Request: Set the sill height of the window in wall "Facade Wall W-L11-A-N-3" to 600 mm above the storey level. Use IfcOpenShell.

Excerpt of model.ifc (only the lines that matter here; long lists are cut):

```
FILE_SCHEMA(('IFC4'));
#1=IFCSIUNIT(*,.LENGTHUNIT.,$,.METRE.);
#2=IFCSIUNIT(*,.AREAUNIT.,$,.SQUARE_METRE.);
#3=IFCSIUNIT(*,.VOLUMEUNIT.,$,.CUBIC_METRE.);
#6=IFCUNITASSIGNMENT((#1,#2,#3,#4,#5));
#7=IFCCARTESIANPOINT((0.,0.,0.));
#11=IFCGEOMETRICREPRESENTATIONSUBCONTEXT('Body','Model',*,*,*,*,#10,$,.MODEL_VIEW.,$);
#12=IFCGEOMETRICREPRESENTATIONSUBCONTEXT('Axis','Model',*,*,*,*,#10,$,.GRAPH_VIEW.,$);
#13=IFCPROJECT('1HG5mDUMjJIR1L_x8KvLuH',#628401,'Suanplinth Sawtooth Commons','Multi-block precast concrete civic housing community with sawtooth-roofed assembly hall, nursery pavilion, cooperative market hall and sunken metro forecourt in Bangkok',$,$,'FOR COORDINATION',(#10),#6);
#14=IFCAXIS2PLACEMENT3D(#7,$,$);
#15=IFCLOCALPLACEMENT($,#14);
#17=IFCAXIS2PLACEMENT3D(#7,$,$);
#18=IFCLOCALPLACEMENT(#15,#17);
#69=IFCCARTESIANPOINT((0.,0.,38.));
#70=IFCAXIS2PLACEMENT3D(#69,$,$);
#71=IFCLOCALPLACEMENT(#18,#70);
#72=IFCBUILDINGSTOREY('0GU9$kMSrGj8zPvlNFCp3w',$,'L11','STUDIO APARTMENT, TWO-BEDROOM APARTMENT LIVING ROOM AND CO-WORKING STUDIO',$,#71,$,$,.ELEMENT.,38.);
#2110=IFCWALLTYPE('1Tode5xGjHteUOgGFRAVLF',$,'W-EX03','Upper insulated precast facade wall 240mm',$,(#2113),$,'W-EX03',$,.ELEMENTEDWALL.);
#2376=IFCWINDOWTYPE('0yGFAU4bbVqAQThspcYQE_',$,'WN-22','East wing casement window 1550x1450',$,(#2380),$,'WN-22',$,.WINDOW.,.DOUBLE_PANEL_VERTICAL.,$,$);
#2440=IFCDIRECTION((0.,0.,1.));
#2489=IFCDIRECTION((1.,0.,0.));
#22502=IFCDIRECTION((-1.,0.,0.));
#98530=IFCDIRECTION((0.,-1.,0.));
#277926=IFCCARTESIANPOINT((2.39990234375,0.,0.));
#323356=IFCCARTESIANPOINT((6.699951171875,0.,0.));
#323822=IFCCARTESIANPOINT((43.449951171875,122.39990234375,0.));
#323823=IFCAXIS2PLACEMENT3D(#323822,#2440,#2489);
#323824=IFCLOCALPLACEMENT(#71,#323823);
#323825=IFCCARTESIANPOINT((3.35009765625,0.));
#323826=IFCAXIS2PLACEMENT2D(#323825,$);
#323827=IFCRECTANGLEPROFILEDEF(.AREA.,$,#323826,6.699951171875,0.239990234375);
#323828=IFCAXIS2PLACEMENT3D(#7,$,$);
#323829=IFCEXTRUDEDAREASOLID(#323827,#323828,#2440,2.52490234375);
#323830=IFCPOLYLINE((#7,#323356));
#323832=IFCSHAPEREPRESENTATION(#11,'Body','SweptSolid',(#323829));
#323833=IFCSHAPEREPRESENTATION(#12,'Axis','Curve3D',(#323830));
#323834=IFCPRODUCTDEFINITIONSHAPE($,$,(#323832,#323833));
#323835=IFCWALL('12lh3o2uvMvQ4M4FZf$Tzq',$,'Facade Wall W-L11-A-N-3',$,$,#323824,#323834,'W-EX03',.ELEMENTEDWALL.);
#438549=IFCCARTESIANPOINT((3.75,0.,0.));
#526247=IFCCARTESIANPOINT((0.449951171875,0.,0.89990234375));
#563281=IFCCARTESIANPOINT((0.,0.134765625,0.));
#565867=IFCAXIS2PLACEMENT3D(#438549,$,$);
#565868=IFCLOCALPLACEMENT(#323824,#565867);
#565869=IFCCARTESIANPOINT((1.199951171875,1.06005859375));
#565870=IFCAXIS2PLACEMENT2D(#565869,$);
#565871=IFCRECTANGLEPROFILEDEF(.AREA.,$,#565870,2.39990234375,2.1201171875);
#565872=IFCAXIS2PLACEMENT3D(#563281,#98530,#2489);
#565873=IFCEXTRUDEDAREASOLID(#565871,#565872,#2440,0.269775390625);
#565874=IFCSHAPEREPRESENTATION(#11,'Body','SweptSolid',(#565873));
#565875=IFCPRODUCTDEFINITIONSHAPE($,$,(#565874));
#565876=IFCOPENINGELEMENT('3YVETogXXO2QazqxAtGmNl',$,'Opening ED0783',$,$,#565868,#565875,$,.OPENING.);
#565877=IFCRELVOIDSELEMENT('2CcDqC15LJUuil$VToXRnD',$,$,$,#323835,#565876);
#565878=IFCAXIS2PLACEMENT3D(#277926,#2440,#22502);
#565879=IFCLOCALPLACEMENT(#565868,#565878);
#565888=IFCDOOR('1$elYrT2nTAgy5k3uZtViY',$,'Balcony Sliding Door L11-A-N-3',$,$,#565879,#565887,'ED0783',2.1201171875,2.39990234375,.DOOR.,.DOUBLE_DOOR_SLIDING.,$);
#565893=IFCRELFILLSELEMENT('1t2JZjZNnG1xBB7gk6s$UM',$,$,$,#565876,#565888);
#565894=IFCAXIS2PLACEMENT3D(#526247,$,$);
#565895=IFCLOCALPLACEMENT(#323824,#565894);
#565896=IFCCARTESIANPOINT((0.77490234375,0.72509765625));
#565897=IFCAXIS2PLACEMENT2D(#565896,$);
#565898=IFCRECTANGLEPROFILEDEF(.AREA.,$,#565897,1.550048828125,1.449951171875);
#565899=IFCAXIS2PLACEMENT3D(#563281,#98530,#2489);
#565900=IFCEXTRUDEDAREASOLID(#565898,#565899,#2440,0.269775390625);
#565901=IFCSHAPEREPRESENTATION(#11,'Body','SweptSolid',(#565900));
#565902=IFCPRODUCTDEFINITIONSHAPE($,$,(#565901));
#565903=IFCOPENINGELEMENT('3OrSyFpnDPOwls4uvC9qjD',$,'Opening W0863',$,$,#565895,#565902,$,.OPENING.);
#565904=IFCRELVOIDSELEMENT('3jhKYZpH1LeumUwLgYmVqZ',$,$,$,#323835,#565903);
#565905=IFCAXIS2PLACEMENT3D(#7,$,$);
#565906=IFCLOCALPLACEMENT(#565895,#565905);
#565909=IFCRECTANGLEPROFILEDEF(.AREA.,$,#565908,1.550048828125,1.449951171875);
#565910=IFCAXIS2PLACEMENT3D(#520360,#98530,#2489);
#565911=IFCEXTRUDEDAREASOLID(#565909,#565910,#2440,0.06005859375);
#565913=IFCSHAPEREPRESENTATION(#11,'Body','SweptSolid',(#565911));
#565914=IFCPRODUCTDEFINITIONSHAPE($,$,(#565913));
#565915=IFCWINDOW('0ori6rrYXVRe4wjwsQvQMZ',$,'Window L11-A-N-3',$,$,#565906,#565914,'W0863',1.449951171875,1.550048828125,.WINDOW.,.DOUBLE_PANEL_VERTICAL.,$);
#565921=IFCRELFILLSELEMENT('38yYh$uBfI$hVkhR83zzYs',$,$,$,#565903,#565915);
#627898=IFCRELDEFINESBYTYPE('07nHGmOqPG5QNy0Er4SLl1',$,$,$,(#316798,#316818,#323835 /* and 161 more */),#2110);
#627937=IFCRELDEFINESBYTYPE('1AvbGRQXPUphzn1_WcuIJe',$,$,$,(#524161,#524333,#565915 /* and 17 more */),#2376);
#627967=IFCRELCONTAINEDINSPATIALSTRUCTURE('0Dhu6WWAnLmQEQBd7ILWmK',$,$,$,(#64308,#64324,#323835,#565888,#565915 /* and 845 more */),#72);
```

```python
import numpy as np
import ifcopenshell
import ifcopenshell.api.geometry
import ifcopenshell.geom
import ifcopenshell.util.element
import ifcopenshell.util.placement
import ifcopenshell.util.shape
import ifcopenshell.util.unit

model = ifcopenshell.open("model.ifc")
unit_scale = ifcopenshell.util.unit.calculate_unit_scale(model)

window = model.by_guid("0ori6rrYXVRe4wjwsQvQMZ")
opening = window.FillsVoids[0].RelatingOpeningElement
storey = ifcopenshell.util.element.get_container(window, ifc_class="IfcBuildingStorey")
level = ifcopenshell.util.placement.get_local_placement(storey.ObjectPlacement)[2, 3]

# The opening's origin need not be at the sill, so measure its lowest point.
shape = ifcopenshell.geom.create_shape(ifcopenshell.geom.settings(), opening)
bottom = ifcopenshell.util.shape.get_shape_bottom_elevation(shape, shape.geometry) / unit_scale
dz = level + 0.6 / unit_scale - bottom

shift = np.array([0.0, 0.0, dz])
# The window is placed relative to its opening, so it follows when the opening moves.
matrix = ifcopenshell.util.placement.get_local_placement(opening.ObjectPlacement)
matrix[:3, 3] += shift
ifcopenshell.api.geometry.edit_object_placement(
    model, product=opening, matrix=matrix, is_si=False, should_transform_children=True
)

print(f"moved by {dz * unit_scale:+.3f} m")

model.write("model_updated.ifc")
```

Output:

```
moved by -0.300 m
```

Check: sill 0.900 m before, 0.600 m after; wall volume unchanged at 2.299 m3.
